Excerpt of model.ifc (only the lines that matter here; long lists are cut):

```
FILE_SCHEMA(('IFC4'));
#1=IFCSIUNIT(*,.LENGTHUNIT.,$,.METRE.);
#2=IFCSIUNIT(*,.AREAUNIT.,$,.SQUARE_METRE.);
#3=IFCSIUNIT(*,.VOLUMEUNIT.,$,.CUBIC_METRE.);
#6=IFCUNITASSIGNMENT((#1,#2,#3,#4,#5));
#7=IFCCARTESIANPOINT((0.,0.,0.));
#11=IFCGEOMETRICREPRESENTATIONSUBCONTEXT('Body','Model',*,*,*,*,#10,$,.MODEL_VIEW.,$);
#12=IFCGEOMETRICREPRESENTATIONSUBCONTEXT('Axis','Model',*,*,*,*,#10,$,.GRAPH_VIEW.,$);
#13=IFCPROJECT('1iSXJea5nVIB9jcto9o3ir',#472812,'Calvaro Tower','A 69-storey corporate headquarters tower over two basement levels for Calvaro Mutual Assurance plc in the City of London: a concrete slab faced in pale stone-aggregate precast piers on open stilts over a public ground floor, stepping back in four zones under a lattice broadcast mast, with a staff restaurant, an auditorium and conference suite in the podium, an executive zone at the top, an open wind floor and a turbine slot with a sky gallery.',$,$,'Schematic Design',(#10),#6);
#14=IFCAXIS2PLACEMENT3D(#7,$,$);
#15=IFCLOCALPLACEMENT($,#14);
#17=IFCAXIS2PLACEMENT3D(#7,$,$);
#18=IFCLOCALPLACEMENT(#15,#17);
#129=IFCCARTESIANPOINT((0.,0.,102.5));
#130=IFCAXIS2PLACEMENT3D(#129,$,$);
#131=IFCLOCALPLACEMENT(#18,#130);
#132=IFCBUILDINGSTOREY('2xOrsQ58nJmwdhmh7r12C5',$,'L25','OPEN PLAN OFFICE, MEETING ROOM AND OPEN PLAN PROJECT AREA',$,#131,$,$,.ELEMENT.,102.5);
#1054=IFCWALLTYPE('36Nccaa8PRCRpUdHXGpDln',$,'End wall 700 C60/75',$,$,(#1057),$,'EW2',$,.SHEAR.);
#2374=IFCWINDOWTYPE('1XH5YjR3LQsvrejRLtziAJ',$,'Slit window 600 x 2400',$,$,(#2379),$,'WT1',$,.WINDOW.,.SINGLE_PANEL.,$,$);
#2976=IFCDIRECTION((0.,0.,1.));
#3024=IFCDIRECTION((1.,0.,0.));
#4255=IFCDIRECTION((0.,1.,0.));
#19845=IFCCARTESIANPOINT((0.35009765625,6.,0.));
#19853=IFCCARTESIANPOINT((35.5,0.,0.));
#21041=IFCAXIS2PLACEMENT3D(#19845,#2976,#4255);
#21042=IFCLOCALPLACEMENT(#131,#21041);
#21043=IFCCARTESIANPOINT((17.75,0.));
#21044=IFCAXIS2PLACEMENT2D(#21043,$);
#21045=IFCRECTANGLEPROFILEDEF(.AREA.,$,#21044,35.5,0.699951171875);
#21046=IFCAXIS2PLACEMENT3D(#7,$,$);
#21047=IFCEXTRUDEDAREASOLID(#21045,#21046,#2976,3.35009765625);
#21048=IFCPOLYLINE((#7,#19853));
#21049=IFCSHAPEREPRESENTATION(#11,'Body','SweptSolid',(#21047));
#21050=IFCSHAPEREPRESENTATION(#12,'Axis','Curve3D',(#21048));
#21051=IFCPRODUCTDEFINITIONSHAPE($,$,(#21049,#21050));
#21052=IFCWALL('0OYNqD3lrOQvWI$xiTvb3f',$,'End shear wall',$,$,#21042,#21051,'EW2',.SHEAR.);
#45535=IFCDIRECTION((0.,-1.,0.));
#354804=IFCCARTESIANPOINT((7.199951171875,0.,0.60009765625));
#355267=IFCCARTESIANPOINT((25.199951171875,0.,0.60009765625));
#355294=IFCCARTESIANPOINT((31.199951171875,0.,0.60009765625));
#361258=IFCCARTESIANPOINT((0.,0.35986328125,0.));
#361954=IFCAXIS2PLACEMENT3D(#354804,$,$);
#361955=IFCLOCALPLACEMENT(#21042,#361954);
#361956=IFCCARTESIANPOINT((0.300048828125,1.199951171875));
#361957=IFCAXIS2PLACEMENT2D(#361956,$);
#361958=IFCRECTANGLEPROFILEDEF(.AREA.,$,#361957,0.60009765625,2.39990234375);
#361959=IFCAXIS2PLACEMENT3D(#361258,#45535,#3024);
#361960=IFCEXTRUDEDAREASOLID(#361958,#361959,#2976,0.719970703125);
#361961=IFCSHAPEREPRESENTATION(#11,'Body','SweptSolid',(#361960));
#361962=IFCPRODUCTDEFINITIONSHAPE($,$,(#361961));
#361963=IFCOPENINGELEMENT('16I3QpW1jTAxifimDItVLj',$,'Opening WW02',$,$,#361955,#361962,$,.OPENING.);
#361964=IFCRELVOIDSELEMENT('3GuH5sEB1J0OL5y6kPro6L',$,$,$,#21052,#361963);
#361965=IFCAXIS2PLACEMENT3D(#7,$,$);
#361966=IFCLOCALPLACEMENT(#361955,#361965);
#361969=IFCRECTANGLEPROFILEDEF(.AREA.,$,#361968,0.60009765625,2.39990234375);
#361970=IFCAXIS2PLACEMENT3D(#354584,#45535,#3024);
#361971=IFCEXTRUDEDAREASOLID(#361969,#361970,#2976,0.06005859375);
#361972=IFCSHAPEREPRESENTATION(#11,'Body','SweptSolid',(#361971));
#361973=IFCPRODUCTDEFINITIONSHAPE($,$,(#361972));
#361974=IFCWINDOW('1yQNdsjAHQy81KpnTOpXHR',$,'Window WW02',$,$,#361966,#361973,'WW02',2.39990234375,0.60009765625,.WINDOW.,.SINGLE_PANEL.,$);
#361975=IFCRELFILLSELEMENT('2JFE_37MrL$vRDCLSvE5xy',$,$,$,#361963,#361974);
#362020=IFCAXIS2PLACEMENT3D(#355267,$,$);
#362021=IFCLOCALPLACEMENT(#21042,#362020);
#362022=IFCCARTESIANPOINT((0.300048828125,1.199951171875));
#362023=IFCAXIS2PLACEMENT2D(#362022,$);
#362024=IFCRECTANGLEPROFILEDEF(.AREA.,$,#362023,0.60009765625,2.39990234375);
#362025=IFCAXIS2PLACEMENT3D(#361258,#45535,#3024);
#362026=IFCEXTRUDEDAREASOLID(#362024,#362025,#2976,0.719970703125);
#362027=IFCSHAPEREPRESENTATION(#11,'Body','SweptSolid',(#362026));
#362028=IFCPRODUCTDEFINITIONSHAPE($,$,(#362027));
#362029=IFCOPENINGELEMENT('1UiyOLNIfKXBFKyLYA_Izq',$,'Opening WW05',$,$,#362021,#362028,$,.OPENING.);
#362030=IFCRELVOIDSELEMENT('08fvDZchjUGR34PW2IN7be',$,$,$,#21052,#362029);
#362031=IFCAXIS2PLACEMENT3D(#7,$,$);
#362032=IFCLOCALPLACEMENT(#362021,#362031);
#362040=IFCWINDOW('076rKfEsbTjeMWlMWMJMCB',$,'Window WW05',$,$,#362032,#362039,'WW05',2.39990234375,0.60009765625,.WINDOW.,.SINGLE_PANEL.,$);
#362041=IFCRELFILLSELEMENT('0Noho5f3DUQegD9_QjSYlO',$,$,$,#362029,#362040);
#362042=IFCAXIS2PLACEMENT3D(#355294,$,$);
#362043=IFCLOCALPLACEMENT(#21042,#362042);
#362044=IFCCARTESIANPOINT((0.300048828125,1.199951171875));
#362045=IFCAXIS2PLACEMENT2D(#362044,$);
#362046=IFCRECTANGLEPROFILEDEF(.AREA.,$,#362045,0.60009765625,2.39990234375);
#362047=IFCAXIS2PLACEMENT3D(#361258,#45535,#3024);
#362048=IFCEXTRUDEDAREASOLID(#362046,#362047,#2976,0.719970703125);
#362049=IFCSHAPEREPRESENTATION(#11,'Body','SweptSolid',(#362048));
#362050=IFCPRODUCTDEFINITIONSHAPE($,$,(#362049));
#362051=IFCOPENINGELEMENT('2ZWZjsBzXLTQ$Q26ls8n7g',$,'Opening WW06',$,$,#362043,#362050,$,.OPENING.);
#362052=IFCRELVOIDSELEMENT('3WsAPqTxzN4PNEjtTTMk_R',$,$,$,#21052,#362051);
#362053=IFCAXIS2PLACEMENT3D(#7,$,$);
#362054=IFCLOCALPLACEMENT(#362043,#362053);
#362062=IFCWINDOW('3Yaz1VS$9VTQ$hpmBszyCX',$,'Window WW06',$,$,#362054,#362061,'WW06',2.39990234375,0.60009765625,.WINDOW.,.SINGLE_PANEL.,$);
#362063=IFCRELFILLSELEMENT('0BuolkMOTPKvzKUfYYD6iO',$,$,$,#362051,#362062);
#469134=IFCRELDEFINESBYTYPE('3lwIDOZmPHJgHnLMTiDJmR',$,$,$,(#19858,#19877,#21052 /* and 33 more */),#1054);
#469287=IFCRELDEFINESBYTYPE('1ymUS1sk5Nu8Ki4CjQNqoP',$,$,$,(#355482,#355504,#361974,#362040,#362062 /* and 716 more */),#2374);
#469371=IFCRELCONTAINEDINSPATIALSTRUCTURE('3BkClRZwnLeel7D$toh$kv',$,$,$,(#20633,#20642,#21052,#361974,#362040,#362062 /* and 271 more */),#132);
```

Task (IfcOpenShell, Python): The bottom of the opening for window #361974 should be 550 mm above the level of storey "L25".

```python
import numpy as np
import ifcopenshell
import ifcopenshell.api.geometry
import ifcopenshell.geom
import ifcopenshell.util.element
import ifcopenshell.util.placement
import ifcopenshell.util.shape
import ifcopenshell.util.unit

model = ifcopenshell.open("model.ifc")
unit_scale = ifcopenshell.util.unit.calculate_unit_scale(model)

window = model.by_id(361974)
opening = window.FillsVoids[0].RelatingOpeningElement
storey = ifcopenshell.util.element.get_container(window, ifc_class="IfcBuildingStorey")
level = ifcopenshell.util.placement.get_local_placement(storey.ObjectPlacement)[2, 3]

# The opening's origin need not be at the sill, so measure its lowest point.
shape = ifcopenshell.geom.create_shape(ifcopenshell.geom.settings(), opening)
bottom = ifcopenshell.util.shape.get_shape_bottom_elevation(shape, shape.geometry) / unit_scale
dz = level + 0.55 - bottom

shift = np.array([0.0, 0.0, dz])
# The window is placed relative to its opening, so it follows when the opening moves.
matrix = ifcopenshell.util.placement.get_local_placement(opening.ObjectPlacement)
matrix[:3, 3] += shift
ifcopenshell.api.geometry.edit_object_placement(
    model, product=opening, matrix=matrix, is_si=False, should_transform_children=True
)

print(f"moved by {dz * unit_scale:+.3f} m")

model.write("model_edited.ifc")
```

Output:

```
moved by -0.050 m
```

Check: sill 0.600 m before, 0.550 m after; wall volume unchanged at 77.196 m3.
